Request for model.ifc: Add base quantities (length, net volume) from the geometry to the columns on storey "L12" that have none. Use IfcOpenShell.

First a look at what the model holds.

```python
import ifcopenshell
import ifcopenshell.util.element
import ifcopenshell.util.unit

model = ifcopenshell.open("model.ifc")
print(model.schema)
for unit_type in ("LENGTHUNIT", "AREAUNIT", "VOLUMEUNIT"):
    print(unit_type, ifcopenshell.util.unit.calculate_unit_scale(model, unit_type))
storey = next(s for s in model.by_type("IfcBuildingStorey") if s.Name == "L12")
columns = [e for e in ifcopenshell.util.element.get_decomposition(storey) if e.is_a("IfcColumn")]
for e in sorted(columns, key=lambda e: e.id()):
    print(e.id(), e.is_a(), e.Name, list(ifcopenshell.util.element.get_psets(e, qtos_only=True)), sep=" | ")
```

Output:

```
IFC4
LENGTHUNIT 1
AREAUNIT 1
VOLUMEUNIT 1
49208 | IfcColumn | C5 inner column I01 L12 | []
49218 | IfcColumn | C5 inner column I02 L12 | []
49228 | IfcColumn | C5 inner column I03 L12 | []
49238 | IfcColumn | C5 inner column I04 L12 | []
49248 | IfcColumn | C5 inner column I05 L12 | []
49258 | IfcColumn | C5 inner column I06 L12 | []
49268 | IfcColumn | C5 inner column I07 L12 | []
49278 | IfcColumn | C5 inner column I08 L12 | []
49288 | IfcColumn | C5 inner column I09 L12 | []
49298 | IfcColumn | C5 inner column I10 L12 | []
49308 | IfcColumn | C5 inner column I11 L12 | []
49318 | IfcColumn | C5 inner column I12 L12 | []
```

```python
import ifcopenshell
import ifcopenshell.api.pset
import ifcopenshell.geom
import ifcopenshell.util.element
import ifcopenshell.util.shape
import ifcopenshell.util.unit

model = ifcopenshell.open("model.ifc")
unit_scale = ifcopenshell.util.unit.calculate_unit_scale(model)
volume_scale = ifcopenshell.util.unit.calculate_unit_scale(model, "VOLUMEUNIT")
settings = ifcopenshell.geom.settings()

storey = next(s for s in model.by_type("IfcBuildingStorey") if s.Name == "L12")
columns = [e for e in ifcopenshell.util.element.get_decomposition(storey) if e.is_a("IfcColumn")]

for e in sorted(columns, key=lambda e: e.id()):
    if ifcopenshell.util.element.get_psets(e, qtos_only=True, should_inherit=False):
        continue
    # Geometry comes back in metres, in the element's own axes.
    shape = ifcopenshell.geom.create_shape(settings, e)
    values = {
        "Length": ifcopenshell.util.shape.get_z(shape.geometry) / unit_scale,
        "NetVolume": ifcopenshell.util.shape.get_volume(shape.geometry) / volume_scale,
    }
    qto = ifcopenshell.api.pset.add_qto(model, product=e, name="Qto_ColumnBaseQuantities")
    ifcopenshell.api.pset.edit_qto(model, qto=qto, properties=values)
    print(e.id(), {k: round(v, 3) for k, v in values.items()})

model.write("model_v2.ifc")
```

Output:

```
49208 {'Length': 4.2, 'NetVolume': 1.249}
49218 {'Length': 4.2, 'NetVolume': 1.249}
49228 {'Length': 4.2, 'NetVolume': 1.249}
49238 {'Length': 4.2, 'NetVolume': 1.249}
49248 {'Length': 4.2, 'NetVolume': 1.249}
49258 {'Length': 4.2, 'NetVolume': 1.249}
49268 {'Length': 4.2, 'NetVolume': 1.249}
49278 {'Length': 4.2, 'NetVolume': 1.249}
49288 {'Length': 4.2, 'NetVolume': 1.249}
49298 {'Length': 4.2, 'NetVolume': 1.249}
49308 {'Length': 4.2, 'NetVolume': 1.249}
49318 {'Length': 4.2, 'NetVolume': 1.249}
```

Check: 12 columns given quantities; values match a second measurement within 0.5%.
